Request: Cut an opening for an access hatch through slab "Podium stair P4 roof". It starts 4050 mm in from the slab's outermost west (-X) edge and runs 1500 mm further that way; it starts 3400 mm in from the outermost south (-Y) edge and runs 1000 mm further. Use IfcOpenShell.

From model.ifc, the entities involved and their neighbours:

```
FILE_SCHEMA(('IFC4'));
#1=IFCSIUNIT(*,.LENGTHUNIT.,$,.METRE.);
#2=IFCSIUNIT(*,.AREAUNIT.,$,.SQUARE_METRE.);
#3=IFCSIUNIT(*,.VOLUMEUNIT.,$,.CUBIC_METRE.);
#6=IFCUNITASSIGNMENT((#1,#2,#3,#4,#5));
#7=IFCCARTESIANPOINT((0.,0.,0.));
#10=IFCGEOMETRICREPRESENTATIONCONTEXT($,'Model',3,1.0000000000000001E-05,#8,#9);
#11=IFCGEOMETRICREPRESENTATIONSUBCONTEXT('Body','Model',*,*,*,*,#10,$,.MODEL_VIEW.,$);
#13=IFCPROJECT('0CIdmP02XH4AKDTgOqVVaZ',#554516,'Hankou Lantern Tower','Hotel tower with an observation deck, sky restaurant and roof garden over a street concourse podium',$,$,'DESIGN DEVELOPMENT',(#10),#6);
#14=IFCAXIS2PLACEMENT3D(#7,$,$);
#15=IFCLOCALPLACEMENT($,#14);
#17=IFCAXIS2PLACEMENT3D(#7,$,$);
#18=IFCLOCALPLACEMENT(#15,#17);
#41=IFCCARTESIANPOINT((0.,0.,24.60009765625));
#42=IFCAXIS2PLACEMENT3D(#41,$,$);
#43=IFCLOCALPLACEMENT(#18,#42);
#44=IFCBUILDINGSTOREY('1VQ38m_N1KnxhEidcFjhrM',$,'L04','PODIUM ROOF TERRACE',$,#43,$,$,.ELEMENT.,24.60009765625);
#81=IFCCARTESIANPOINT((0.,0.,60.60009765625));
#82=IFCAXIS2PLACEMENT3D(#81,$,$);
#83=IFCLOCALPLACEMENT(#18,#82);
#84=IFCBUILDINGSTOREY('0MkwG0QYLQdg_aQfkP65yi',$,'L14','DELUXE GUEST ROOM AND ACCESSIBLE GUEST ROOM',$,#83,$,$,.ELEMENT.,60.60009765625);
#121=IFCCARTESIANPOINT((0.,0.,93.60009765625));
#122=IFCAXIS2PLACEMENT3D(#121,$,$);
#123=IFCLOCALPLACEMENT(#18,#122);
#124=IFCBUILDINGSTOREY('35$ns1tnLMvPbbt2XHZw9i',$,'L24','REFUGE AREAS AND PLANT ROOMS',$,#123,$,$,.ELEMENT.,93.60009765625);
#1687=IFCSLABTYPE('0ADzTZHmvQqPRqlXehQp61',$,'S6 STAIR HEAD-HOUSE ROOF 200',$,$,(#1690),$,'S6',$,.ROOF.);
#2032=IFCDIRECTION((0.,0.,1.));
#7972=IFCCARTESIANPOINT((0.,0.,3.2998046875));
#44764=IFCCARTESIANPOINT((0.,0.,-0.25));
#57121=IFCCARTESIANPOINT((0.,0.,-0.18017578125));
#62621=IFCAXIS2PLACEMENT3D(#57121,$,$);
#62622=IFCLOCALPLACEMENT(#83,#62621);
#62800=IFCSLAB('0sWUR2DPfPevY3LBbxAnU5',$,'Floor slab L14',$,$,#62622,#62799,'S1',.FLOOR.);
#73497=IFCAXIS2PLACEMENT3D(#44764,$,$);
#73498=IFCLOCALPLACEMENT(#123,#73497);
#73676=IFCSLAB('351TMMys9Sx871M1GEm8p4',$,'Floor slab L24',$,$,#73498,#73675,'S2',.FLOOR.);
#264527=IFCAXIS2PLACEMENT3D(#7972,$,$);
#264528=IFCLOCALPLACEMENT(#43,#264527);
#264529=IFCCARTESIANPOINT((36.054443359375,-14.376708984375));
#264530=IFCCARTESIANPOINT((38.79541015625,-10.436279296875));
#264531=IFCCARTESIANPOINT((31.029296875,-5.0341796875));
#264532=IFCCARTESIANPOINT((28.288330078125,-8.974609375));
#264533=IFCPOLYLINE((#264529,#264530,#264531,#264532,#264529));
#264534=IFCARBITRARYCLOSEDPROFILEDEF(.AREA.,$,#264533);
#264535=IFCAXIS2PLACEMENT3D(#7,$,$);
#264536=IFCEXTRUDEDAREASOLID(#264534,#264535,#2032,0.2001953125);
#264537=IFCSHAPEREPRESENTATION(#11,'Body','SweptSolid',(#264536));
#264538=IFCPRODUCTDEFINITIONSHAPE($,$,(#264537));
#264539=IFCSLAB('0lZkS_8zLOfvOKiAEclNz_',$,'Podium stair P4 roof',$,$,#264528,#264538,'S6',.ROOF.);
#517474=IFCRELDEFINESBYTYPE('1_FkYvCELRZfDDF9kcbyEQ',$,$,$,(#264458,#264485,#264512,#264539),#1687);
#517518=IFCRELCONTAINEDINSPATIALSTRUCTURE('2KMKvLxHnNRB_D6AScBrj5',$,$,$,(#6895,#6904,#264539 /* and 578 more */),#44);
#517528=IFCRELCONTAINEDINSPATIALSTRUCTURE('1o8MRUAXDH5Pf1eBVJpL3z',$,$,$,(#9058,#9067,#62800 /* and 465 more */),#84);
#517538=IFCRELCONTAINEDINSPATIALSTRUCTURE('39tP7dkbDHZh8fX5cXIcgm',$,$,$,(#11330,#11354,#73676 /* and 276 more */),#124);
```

```python
import numpy as np
import ifcopenshell
import ifcopenshell.api.feature
import ifcopenshell.api.geometry
import ifcopenshell.api.root
import ifcopenshell.geom
import ifcopenshell.util.placement
import ifcopenshell.util.representation
import ifcopenshell.util.shape
import ifcopenshell.util.unit

model = ifcopenshell.open("model.ifc")
unit_scale = ifcopenshell.util.unit.calculate_unit_scale(model)
settings = ifcopenshell.geom.settings()


def volume(element):
    """Net volume in cubic metres, openings subtracted."""
    shape = ifcopenshell.geom.create_shape(settings, element)
    return ifcopenshell.util.shape.get_volume(shape.geometry)


slab = model.by_id(264539)
before = volume(slab)

# Extent in the slab's own axes, in metres. The edges named are its -X and -Y sides.
slab_shape = ifcopenshell.geom.create_shape(settings, slab)
vertices = ifcopenshell.util.shape.get_vertices(slab_shape.geometry)
x_min, y_min, bottom = vertices.min(axis=0)
top = vertices[:, 2].max()

opening = ifcopenshell.api.root.create_entity(model, ifc_class="IfcOpeningElement", name="Access hatch opening", predefined_type="OPENING")
context = ifcopenshell.util.representation.get_context(model, "Model", "Body", "MODEL_VIEW")
width, depth = 1.5, 1
outline = [(0.0, 0.0), (width, 0.0), (width, depth), (0.0, depth), (0.0, 0.0)]
# Overshoot both faces by 50 mm so the cut is clean.
shape = ifcopenshell.api.geometry.add_slab_representation(
    model, context=context, depth=top - bottom + 0.1, polyline=outline
)
ifcopenshell.api.geometry.assign_representation(model, product=opening, representation=shape)

matrix = ifcopenshell.util.placement.get_local_placement(slab.ObjectPlacement)
matrix[:, 3] = matrix @ np.append(np.array([x_min + 4.05, y_min + 3.4, bottom - 0.05]) / unit_scale, 1.0)
ifcopenshell.api.geometry.edit_object_placement(model, product=opening, matrix=matrix, is_si=False)
ifcopenshell.api.feature.add_feature(model, feature=opening, element=slab)

after = volume(slab)

print(f"slab volume {before:.3f} -> {after:.3f} m3")

model.write("model_edited.ifc")
```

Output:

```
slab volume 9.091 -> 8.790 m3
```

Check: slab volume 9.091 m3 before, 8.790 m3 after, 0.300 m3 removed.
